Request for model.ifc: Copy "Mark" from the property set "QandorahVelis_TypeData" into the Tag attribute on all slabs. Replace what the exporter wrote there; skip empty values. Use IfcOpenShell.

First a look at what the model holds.

```python
import ifcopenshell
import ifcopenshell.util.element

model = ifcopenshell.open("model.ifc")
print(model.schema)
slabs = model.by_type("IfcSlab")
print(len(slabs), "slabs")
for e in slabs[:8]:
    source = ifcopenshell.util.element.get_pset(e, "QandorahVelis_TypeData", "Mark")
    target = e.Tag
    print(e.id(), repr(source), repr(target), sep=" | ")
```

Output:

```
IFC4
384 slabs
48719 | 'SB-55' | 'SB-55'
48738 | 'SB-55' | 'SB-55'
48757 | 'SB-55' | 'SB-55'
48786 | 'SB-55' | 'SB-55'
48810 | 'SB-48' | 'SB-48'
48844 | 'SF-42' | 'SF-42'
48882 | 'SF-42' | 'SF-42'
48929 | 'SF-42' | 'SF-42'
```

```python
import ifcopenshell
import ifcopenshell.util.element

model = ifcopenshell.open("model.ifc")

count = 0
for e in model.by_type("IfcSlab"):
    value = ifcopenshell.util.element.get_pset(e, "QandorahVelis_TypeData", "Mark")
    current = e.Tag
    if not value or not value.strip() or current == value:
        continue
    e.Tag = value
    count += 1

print(count, "slabs updated")

model.write("model_v2.ifc")
```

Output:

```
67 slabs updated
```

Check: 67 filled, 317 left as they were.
